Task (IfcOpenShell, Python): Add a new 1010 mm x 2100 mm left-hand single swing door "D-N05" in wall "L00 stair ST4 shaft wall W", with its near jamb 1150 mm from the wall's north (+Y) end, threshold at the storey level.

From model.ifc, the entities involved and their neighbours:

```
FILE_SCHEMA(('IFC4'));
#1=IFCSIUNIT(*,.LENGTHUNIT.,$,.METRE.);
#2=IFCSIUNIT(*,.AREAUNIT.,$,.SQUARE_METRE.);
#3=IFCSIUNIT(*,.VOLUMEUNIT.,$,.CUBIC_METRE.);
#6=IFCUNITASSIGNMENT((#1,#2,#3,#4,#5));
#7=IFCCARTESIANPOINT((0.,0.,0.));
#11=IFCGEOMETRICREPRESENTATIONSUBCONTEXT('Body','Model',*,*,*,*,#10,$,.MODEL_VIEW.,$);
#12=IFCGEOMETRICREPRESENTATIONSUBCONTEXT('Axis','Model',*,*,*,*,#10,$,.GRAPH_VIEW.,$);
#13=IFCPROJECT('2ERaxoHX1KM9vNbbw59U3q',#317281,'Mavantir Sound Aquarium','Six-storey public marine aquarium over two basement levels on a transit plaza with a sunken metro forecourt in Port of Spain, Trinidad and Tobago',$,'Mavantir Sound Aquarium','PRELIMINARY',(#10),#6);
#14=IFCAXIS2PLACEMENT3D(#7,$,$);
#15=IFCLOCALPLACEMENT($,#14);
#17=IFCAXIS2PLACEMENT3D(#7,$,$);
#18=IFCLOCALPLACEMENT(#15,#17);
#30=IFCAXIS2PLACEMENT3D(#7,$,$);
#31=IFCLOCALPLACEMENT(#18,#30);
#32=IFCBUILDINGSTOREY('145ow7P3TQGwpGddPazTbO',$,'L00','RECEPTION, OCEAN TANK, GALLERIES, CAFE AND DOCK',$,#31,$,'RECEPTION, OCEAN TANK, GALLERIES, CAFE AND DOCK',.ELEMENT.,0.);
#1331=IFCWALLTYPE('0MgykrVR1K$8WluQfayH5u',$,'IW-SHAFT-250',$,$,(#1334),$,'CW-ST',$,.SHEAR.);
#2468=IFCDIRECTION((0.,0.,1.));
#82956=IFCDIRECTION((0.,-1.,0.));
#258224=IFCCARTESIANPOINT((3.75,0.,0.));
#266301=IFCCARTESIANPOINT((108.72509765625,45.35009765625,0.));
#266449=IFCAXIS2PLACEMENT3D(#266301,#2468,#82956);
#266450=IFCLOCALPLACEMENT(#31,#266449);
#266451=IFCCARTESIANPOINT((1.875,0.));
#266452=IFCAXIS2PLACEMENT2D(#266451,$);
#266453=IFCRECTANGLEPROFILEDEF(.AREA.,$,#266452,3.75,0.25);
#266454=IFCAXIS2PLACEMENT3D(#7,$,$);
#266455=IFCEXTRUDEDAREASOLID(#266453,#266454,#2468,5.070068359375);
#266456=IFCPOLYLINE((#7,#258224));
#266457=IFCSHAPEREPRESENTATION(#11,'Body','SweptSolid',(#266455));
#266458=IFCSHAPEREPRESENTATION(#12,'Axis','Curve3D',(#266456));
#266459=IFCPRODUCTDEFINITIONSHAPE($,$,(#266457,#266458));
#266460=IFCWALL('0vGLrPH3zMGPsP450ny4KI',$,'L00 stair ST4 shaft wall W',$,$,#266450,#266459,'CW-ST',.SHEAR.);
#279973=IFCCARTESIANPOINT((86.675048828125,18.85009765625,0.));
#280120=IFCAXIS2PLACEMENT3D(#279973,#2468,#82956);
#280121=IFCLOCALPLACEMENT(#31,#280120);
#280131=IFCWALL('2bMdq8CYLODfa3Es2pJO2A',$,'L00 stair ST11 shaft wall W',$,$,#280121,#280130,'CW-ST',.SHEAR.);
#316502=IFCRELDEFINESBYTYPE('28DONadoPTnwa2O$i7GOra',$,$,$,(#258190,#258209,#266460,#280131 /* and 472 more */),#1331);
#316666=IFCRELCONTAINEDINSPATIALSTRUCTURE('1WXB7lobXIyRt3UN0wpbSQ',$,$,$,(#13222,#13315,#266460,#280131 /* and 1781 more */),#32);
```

```python
import numpy as np
import ifcopenshell
import ifcopenshell.api.feature
import ifcopenshell.api.geometry
import ifcopenshell.api.root
import ifcopenshell.api.spatial
import ifcopenshell.geom
import ifcopenshell.util.element
import ifcopenshell.util.placement
import ifcopenshell.util.representation
import ifcopenshell.util.shape
import ifcopenshell.util.unit

model = ifcopenshell.open("model.ifc")
unit_scale = ifcopenshell.util.unit.calculate_unit_scale(model)
settings = ifcopenshell.geom.settings()


def volume(element):
    """Net volume in cubic metres, openings subtracted."""
    shape = ifcopenshell.geom.create_shape(settings, element)
    return ifcopenshell.util.shape.get_volume(shape.geometry)


wall = model.by_guid("0vGLrPH3zMGPsP450ny4KI")
storey = ifcopenshell.util.element.get_container(wall, ifc_class="IfcBuildingStorey")
context = ifcopenshell.util.representation.get_context(model, "Model", "Body", "MODEL_VIEW")
before = volume(wall)

width, height, from_end, sill = 1.01, 2.1, 1.15, 0.0  # metres

# The wall runs along its own X axis, and the end named is its -X end.
wall_shape = ifcopenshell.geom.create_shape(settings, wall)
x, y, z = ifcopenshell.util.shape.get_vertices(wall_shape.geometry).T
start = x.min() + from_end
face, thickness = float(y.min()), float(y.max() - y.min())
wall_matrix = ifcopenshell.util.placement.get_local_placement(wall.ObjectPlacement)
level = ifcopenshell.util.placement.get_local_placement(storey.ObjectPlacement)[2, 3]


def in_wall(x, y):
    """Placement at x, y metres in the wall's axes, at sill height."""
    matrix = wall_matrix.copy()
    matrix[:, 3] = wall_matrix @ np.array([x / unit_scale, y / unit_scale, 0.0, 1.0])
    matrix[2, 3] = level + sill / unit_scale
    return matrix


# Opening: a box that overshoots both wall faces by 50 mm.
opening = ifcopenshell.api.root.create_entity(model, ifc_class="IfcOpeningElement", predefined_type="OPENING")
box = ifcopenshell.api.geometry.add_wall_representation(
    model, context=context, length=width, height=height, thickness=thickness + 0.1
)
ifcopenshell.api.geometry.assign_representation(model, product=opening, representation=box)
ifcopenshell.api.geometry.edit_object_placement(model, product=opening, matrix=in_wall(start, face - 0.05), is_si=False)
ifcopenshell.api.feature.add_feature(model, feature=opening, element=wall)

door = ifcopenshell.api.root.create_entity(model, ifc_class="IfcDoor", name="D-N05", predefined_type="DOOR")
door.OverallWidth, door.OverallHeight = width / unit_scale, height / unit_scale
door.OperationType = "SINGLE_SWING_LEFT"
body = ifcopenshell.api.geometry.add_door_representation(
    model,
    context=context,
    overall_width=door.OverallWidth,
    overall_height=door.OverallHeight,
    operation_type="SINGLE_SWING_LEFT",
    lining_properties={"LiningDepth": thickness / unit_scale, "ThresholdDepth": thickness / unit_scale},
)
ifcopenshell.api.geometry.assign_representation(model, product=door, representation=body)
ifcopenshell.api.spatial.assign_container(model, products=[door], relating_structure=storey)
ifcopenshell.api.feature.add_filling(model, opening=opening, element=door)

# The lining spans the wall, so the door starts at the wall face.
ifcopenshell.api.geometry.edit_object_placement(model, product=door, matrix=in_wall(start, face), is_si=False)

after = volume(wall)

print(f"wall volume {before:.3f} -> {after:.3f} m3")

model.write("model_edited.ifc")
```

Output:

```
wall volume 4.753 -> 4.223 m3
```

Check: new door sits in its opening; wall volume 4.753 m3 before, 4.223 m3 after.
